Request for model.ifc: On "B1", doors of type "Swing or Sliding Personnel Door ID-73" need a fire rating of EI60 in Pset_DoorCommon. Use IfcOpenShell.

First a look at what the model holds.

```python
import ifcopenshell
import ifcopenshell.util.element

model = ifcopenshell.open("model.ifc")
print(model.schema)
storey = next(s for s in model.by_type("IfcBuildingStorey") if s.Name == "B1")
doors = [e for e in ifcopenshell.util.element.get_decomposition(storey) if e.is_a("IfcDoor")]
seen = {}
for e in doors:
    element_type = ifcopenshell.util.element.get_type(e)
    key = (element_type.Name if element_type != e and element_type else None, ifcopenshell.util.element.get_pset(e, "Pset_DoorCommon", "FireRating"))
    seen[key] = seen.get(key, 0) + 1
for (name, value), count in sorted(seen.items(), key=str):
    print(count, "x", name, "|", value)
```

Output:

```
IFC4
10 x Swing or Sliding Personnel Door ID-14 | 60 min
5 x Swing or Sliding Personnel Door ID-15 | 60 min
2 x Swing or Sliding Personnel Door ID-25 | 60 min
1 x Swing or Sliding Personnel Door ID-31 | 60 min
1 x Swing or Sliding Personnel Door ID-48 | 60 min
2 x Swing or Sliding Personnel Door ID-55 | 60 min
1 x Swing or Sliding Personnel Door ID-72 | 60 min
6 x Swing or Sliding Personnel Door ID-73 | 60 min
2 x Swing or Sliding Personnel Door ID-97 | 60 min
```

```python
import ifcopenshell
import ifcopenshell.api.pset
import ifcopenshell.util.element

model = ifcopenshell.open("model.ifc")

storey = next(s for s in model.by_type("IfcBuildingStorey") if s.Name == "B1")
doors = [e for e in ifcopenshell.util.element.get_decomposition(storey) if e.is_a("IfcDoor")]

count = 0
for e in doors:
    element_type = ifcopenshell.util.element.get_type(e)
    if element_type in (None, e) or element_type.Name != "Swing or Sliding Personnel Door ID-73":
        continue
    # add_pset returns the element's existing set when there is one.
    pset = ifcopenshell.api.pset.add_pset(model, product=e, name="Pset_DoorCommon")
    ifcopenshell.api.pset.edit_pset(model, pset=pset, properties={"FireRating": "EI60"})
    count += 1

print(count, "doors updated")

model.write("model_edited.ifc")
```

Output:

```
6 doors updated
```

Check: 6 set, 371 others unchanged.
